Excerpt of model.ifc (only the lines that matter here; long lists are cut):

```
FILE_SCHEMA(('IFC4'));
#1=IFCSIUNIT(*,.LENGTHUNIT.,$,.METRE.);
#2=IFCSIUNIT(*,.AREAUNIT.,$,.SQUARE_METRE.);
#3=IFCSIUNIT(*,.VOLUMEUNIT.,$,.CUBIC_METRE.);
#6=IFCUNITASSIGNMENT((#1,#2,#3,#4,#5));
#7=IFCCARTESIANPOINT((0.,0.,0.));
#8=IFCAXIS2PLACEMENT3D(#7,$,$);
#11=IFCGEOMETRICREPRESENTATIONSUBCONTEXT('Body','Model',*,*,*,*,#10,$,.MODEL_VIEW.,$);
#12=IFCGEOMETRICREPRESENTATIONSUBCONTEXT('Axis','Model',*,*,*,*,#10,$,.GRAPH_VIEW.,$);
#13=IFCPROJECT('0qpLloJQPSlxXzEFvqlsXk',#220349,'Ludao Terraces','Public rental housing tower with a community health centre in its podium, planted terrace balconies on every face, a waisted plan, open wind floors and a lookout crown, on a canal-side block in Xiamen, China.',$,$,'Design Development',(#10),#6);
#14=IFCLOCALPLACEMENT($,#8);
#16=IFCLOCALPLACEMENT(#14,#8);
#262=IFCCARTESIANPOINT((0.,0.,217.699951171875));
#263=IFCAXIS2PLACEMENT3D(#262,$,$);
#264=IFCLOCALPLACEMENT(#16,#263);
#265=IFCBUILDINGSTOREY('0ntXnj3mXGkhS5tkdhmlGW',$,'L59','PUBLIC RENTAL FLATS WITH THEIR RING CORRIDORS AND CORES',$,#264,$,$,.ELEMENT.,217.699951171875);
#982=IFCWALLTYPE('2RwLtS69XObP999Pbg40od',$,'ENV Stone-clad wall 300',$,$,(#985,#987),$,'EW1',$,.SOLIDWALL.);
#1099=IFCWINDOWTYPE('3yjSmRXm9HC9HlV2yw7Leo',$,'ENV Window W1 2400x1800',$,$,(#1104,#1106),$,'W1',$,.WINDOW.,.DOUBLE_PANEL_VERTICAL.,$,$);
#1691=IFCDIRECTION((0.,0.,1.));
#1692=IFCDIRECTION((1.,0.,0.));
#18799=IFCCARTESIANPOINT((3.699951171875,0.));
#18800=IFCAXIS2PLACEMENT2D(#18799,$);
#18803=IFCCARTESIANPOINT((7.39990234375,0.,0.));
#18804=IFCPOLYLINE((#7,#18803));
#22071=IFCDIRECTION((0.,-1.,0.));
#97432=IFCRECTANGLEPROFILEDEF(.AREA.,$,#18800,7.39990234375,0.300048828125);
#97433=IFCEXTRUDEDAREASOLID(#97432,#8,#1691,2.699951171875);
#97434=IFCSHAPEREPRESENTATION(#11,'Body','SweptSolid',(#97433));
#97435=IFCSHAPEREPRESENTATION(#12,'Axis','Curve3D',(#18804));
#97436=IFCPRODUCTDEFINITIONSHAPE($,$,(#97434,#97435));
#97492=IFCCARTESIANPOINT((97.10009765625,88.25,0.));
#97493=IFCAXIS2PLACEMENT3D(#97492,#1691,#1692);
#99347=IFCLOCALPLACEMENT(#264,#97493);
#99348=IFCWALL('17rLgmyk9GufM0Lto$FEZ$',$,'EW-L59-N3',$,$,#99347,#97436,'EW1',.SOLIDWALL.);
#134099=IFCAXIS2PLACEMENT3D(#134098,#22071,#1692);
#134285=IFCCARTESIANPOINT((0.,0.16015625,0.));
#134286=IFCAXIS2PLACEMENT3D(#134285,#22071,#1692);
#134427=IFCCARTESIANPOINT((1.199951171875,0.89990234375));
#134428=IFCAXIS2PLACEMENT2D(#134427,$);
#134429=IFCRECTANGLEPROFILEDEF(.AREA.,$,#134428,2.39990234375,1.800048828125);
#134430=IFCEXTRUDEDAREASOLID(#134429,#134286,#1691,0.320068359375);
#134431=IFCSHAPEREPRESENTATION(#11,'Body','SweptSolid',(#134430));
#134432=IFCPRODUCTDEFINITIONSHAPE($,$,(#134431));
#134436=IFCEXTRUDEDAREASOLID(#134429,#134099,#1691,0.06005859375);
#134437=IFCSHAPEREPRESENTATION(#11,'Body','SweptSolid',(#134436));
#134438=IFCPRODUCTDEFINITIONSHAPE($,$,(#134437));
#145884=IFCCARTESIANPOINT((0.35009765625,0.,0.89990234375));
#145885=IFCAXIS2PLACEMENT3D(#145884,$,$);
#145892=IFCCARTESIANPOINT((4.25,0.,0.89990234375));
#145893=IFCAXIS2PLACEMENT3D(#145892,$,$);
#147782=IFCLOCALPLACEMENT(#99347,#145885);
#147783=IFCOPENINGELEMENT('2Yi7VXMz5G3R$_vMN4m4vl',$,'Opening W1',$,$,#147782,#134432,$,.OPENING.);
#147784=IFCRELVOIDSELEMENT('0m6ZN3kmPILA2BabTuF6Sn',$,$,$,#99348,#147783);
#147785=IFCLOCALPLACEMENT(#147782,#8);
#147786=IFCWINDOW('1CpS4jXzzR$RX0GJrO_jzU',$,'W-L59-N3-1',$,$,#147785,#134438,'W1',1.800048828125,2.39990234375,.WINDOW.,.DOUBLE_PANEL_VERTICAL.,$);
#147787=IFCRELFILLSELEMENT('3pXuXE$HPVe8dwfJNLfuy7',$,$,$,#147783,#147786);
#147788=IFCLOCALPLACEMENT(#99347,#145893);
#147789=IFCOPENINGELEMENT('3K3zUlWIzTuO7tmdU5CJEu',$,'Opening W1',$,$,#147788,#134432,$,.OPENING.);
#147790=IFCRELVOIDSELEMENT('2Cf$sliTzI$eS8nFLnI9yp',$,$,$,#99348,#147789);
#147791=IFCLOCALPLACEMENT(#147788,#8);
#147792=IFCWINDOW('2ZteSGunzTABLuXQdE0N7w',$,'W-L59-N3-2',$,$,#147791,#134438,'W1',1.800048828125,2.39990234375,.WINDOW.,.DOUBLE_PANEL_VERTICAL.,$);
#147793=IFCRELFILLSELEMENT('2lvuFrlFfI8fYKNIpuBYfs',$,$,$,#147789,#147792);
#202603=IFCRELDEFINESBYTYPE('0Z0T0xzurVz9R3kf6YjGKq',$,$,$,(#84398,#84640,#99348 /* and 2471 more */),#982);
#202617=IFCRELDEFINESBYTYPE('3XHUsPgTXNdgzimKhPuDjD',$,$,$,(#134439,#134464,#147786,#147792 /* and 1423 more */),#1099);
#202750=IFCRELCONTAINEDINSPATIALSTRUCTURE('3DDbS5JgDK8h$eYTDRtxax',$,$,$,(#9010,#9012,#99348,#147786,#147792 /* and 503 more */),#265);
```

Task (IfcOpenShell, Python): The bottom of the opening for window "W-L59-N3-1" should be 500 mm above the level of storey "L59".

```python
import numpy as np
import ifcopenshell
import ifcopenshell.api.geometry
import ifcopenshell.geom
import ifcopenshell.util.element
import ifcopenshell.util.placement
import ifcopenshell.util.shape
import ifcopenshell.util.unit

model = ifcopenshell.open("model.ifc")
unit_scale = ifcopenshell.util.unit.calculate_unit_scale(model)

window = model.by_id(147786)
opening = window.FillsVoids[0].RelatingOpeningElement
storey = ifcopenshell.util.element.get_container(window, ifc_class="IfcBuildingStorey")
level = ifcopenshell.util.placement.get_local_placement(storey.ObjectPlacement)[2, 3]

# The opening's origin need not be at the sill, so measure its lowest point.
shape = ifcopenshell.geom.create_shape(ifcopenshell.geom.settings(), opening)
bottom = ifcopenshell.util.shape.get_shape_bottom_elevation(shape, shape.geometry) / unit_scale
dz = level + 0.5 - bottom

shift = np.array([0.0, 0.0, dz])
# The window is placed relative to its opening, so it follows when the opening moves.
matrix = ifcopenshell.util.placement.get_local_placement(opening.ObjectPlacement)
matrix[:3, 3] += shift
ifcopenshell.api.geometry.edit_object_placement(
    model, product=opening, matrix=matrix, is_si=False, should_transform_children=True
)

print(f"moved by {dz * unit_scale:+.3f} m")

model.write("model_v2.ifc")
```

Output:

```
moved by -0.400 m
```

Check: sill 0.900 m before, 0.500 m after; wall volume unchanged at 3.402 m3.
